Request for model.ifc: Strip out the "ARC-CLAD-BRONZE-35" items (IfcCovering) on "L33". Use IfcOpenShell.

First a look at what the model holds.

```python
import ifcopenshell
import ifcopenshell.util.element

model = ifcopenshell.open("model.ifc")
print(model.schema)
storey = next(s for s in model.by_type("IfcBuildingStorey") if s.Name == "L33")
coverings = [e for e in ifcopenshell.util.element.get_decomposition(storey) if e.is_a("IfcCovering")]
seen = {}
for e in coverings:
    element_type = ifcopenshell.util.element.get_type(e)
    name = element_type.Name if element_type not in (None, e) else None
    seen[name] = seen.get(name, 0) + 1
for name, count in sorted(seen.items(), key=str):
    print(count, "x", name)
```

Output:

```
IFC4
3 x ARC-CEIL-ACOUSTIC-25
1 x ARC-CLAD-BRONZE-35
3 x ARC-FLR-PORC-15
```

```python
import ifcopenshell
import ifcopenshell.api.root
import ifcopenshell.util.element

model = ifcopenshell.open("model.ifc")

storey = next(s for s in model.by_type("IfcBuildingStorey") if s.Name == "L33")
coverings = [e for e in ifcopenshell.util.element.get_decomposition(storey) if e.is_a("IfcCovering")]
targets = [e for e in coverings if (t := ifcopenshell.util.element.get_type(e)) not in (None, e) and t.Name == "ARC-CLAD-BRONZE-35"]

for e in targets:
    ifcopenshell.api.root.remove_product(model, product=e)
print(len(targets), "removed")

model.write("model-out.ifc")
```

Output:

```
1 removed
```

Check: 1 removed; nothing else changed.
